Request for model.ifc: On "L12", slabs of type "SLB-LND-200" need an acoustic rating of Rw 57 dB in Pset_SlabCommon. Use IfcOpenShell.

First a look at what the model holds.

```python
import ifcopenshell
import ifcopenshell.util.element

model = ifcopenshell.open("model.ifc")
print(model.schema)
storey = next(s for s in model.by_type("IfcBuildingStorey") if s.Name == "L12")
slabs = [e for e in ifcopenshell.util.element.get_decomposition(storey) if e.is_a("IfcSlab")]
seen = {}
for e in slabs:
    element_type = ifcopenshell.util.element.get_type(e)
    key = (element_type.Name if element_type != e and element_type else None, ifcopenshell.util.element.get_pset(e, "Pset_SlabCommon", "AcousticRating"))
    seen[key] = seen.get(key, 0) + 1
for (name, value), count in sorted(seen.items(), key=str):
    print(count, "x", name, "|", value)
```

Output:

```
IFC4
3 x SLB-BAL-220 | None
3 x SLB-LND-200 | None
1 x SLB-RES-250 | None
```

```python
import ifcopenshell
import ifcopenshell.api.pset
import ifcopenshell.util.element

model = ifcopenshell.open("model.ifc")

storey = next(s for s in model.by_type("IfcBuildingStorey") if s.Name == "L12")
slabs = [e for e in ifcopenshell.util.element.get_decomposition(storey) if e.is_a("IfcSlab")]

count = 0
for e in slabs:
    element_type = ifcopenshell.util.element.get_type(e)
    if element_type in (None, e) or element_type.Name != "SLB-LND-200":
        continue
    found = ifcopenshell.util.element.get_pset(e, "Pset_SlabCommon", should_inherit=False)
    if found:
        pset = model.by_id(found["id"])
        if len(ifcopenshell.util.element.get_elements_by_pset(pset)) > 1:
            pset = ifcopenshell.api.pset.unshare_pset(model, products=[e], pset=pset)[0]
    else:
        pset = ifcopenshell.api.pset.add_pset(model, product=e, name="Pset_SlabCommon")
    ifcopenshell.api.pset.edit_pset(model, pset=pset, properties={"AcousticRating": "Rw 57 dB"})
    count += 1

print(count, "slabs updated")

model.write("model-out.ifc")
```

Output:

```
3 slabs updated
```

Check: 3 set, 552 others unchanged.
